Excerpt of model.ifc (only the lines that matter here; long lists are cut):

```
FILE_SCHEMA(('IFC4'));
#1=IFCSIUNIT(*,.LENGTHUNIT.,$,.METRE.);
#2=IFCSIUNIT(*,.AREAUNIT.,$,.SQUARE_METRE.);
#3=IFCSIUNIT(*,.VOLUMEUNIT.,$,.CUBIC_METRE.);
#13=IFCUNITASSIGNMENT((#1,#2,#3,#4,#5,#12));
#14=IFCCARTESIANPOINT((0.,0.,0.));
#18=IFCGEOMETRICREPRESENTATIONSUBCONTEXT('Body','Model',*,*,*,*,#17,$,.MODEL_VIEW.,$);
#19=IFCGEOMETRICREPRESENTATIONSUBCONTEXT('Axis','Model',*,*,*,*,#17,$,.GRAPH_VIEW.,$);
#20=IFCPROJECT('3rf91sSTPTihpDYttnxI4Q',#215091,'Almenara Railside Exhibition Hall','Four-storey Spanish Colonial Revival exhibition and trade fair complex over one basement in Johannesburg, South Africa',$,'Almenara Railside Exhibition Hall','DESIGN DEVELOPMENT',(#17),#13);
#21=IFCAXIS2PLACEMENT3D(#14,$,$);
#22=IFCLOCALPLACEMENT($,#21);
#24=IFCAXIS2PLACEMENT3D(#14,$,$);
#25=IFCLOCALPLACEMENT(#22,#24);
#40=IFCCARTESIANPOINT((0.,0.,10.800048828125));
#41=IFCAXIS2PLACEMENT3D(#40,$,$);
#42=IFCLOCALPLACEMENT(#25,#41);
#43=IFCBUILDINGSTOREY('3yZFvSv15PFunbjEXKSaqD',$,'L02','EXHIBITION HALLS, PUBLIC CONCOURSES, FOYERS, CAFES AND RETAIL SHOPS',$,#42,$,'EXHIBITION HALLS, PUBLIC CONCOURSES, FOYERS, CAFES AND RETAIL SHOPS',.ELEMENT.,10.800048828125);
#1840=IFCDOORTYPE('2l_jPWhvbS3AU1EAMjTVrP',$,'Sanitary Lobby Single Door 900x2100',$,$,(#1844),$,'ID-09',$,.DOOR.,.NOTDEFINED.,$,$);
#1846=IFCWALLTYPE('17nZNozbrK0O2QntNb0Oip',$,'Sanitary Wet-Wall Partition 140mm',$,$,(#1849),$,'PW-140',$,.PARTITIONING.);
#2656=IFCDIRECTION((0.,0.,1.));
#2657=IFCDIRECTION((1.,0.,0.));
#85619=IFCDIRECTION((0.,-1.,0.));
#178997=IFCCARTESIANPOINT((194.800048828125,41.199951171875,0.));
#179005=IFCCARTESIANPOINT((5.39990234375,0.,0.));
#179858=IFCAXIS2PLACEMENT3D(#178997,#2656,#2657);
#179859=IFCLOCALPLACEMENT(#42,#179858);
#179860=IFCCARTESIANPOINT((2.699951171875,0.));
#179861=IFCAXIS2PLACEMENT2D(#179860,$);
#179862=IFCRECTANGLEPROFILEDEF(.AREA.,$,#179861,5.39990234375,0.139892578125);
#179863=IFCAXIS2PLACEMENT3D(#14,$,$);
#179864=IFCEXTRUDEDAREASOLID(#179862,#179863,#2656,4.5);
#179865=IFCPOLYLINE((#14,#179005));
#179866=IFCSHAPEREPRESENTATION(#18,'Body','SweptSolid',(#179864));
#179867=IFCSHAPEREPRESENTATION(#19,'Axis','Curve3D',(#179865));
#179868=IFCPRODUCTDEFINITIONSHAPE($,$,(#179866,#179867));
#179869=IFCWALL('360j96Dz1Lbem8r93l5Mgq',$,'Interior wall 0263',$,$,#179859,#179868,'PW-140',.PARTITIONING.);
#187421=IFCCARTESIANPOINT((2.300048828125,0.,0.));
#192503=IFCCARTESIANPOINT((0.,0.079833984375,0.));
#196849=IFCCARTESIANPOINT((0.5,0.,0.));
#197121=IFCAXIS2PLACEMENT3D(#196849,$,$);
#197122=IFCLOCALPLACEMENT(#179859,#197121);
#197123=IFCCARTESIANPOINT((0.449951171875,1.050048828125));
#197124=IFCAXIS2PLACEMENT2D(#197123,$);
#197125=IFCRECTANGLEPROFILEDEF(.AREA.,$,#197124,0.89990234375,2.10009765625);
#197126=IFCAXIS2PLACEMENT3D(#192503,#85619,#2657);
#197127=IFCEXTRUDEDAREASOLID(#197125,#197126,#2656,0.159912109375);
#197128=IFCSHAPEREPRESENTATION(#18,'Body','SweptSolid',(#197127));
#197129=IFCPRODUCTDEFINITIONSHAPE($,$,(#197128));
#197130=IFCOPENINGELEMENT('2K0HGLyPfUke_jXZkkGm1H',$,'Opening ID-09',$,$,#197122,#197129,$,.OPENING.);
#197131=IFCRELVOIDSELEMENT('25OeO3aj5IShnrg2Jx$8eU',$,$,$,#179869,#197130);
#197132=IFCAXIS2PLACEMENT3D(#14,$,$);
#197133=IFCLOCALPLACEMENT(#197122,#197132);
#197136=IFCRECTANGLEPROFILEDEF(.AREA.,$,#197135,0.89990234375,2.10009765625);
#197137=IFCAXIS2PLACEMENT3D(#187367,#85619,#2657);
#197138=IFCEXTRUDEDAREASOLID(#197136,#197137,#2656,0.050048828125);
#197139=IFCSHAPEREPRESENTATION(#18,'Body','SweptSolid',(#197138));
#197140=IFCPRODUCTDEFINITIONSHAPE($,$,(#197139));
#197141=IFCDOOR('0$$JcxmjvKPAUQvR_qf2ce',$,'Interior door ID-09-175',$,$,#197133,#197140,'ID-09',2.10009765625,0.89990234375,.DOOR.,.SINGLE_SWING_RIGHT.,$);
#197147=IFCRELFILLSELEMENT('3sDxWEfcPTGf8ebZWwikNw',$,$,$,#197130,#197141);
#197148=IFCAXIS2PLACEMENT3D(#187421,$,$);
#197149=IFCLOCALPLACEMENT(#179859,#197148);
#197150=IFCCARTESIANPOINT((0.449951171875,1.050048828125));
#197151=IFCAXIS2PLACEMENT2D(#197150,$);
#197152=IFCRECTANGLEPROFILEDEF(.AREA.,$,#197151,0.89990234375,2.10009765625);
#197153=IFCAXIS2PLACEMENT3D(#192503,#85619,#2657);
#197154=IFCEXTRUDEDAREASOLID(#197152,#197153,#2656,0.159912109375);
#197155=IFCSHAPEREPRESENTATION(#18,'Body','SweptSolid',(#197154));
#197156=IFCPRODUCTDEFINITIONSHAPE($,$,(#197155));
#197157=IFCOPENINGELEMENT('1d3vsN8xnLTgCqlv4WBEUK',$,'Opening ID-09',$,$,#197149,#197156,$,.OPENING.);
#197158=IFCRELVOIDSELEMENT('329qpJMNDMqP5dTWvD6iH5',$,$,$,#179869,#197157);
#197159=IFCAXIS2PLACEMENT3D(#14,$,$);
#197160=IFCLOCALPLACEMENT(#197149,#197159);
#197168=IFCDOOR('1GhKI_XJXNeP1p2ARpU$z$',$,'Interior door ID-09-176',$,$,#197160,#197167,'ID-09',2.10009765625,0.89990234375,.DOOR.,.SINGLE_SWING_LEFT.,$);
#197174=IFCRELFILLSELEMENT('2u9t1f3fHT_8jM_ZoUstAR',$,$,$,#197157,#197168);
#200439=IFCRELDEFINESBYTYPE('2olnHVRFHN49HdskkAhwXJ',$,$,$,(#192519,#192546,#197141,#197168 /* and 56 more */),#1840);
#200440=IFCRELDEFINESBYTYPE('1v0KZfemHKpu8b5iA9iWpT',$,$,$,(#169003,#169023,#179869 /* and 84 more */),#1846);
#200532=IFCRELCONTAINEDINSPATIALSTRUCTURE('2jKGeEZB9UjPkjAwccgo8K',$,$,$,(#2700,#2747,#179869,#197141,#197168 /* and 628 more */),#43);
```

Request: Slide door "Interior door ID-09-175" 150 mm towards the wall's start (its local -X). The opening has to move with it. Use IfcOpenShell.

```python
import ifcopenshell
import ifcopenshell.api.geometry
import ifcopenshell.util.placement
import ifcopenshell.util.unit

model = ifcopenshell.open("model.ifc")
unit_scale = ifcopenshell.util.unit.calculate_unit_scale(model)

door = model.by_guid("0$$JcxmjvKPAUQvR_qf2ce")
opening = door.FillsVoids[0].RelatingOpeningElement
wall = opening.VoidsElements[0].RelatingBuildingElement

wall_matrix = ifcopenshell.util.placement.get_local_placement(wall.ObjectPlacement)
shift = wall_matrix[:3, 0] * -0.15 / unit_scale
before = ifcopenshell.util.placement.get_local_placement(door.ObjectPlacement)[:3, 3].copy()

# The door is placed relative to its opening, so it follows when the opening moves.
matrix = ifcopenshell.util.placement.get_local_placement(opening.ObjectPlacement)
matrix[:3, 3] += shift
ifcopenshell.api.geometry.edit_object_placement(
    model, product=opening, matrix=matrix, is_si=False, should_transform_children=True
)

after = ifcopenshell.util.placement.get_local_placement(door.ObjectPlacement)[:3, 3]
print("door moved by", (after - before).round(3) + 0.0)

model.write("model-out.ifc")
```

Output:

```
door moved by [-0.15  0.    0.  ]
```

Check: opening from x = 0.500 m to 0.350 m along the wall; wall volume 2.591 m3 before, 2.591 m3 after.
